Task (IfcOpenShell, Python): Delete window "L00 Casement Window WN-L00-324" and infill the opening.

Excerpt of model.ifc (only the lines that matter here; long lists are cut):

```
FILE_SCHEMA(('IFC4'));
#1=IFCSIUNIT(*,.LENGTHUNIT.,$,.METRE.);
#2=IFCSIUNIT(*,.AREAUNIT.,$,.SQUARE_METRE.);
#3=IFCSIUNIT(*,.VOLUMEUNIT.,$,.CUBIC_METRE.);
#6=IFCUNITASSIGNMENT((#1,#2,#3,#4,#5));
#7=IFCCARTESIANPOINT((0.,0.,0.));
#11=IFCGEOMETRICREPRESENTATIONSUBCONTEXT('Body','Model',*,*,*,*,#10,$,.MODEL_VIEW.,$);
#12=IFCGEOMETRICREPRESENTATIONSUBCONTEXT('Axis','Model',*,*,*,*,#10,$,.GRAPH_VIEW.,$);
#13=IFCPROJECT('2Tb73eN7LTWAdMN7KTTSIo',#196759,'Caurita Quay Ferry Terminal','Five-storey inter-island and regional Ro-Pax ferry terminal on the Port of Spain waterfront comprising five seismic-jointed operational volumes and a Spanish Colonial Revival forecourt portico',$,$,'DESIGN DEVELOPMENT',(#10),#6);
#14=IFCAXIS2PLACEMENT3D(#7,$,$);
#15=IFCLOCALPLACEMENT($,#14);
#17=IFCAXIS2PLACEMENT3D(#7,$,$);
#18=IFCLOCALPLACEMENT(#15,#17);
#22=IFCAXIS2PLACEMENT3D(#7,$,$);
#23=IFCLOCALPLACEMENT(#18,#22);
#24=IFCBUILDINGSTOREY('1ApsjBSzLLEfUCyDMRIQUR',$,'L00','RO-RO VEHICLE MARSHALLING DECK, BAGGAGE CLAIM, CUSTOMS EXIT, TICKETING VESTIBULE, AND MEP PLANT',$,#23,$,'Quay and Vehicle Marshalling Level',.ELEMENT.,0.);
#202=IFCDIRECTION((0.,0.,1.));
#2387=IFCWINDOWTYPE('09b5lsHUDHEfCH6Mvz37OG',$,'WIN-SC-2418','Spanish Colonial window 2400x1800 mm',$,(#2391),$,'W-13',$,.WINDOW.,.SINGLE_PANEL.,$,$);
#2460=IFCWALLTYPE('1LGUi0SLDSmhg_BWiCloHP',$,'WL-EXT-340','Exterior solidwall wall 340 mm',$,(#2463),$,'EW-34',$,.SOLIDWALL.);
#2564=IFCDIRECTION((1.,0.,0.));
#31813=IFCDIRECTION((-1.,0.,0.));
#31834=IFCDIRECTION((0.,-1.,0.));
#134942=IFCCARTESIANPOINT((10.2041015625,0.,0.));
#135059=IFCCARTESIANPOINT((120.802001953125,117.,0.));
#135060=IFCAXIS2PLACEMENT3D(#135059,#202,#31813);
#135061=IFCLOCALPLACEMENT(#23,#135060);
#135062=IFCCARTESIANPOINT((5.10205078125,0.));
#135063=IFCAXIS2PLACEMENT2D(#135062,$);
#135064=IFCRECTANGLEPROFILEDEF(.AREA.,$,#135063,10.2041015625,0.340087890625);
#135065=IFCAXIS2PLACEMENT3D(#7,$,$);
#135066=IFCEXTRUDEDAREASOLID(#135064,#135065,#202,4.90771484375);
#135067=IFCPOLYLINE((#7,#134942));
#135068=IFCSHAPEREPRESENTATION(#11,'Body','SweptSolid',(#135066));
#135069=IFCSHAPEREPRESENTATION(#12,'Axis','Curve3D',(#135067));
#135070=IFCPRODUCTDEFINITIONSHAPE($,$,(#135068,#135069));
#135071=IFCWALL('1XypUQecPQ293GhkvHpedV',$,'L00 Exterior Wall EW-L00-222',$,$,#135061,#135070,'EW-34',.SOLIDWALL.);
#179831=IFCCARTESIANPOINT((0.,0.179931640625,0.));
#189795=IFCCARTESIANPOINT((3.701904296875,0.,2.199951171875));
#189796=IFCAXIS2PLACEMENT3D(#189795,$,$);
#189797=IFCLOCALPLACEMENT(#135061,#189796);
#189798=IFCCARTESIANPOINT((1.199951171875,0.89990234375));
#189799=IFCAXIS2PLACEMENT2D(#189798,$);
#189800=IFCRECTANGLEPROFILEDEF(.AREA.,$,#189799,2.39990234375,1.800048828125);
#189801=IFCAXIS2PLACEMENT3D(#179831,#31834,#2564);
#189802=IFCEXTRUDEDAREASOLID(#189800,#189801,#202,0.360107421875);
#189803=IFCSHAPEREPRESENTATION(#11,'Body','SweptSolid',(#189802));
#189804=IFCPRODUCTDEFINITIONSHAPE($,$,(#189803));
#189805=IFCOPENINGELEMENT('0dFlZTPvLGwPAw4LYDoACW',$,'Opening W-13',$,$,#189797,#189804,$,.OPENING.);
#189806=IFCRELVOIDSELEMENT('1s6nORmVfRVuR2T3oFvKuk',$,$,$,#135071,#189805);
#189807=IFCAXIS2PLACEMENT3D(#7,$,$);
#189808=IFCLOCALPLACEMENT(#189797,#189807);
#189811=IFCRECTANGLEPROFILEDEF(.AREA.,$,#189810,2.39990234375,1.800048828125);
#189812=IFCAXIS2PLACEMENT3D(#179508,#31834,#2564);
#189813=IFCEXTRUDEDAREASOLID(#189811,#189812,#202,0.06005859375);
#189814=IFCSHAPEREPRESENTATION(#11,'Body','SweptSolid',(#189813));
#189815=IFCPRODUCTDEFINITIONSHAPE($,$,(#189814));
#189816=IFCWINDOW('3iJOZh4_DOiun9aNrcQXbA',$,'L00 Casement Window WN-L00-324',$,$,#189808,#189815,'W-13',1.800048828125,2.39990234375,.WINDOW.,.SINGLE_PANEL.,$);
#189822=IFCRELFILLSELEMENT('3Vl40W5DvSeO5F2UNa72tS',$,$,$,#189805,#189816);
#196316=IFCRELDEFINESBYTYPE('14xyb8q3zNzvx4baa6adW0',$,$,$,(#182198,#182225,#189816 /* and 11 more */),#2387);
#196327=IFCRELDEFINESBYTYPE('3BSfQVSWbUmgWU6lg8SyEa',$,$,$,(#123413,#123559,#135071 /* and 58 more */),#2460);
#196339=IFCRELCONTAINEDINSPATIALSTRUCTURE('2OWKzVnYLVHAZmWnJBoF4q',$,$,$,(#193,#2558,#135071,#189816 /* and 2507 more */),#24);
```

```python
import ifcopenshell
import ifcopenshell.api.feature
import ifcopenshell.api.root
import ifcopenshell.geom
import ifcopenshell.util.shape

model = ifcopenshell.open("model.ifc")
settings = ifcopenshell.geom.settings()


def volume(element):
    """Net volume in cubic metres, openings subtracted."""
    shape = ifcopenshell.geom.create_shape(settings, element)
    return ifcopenshell.util.shape.get_volume(shape.geometry)


window = model.by_guid("3iJOZh4_DOiun9aNrcQXbA")
opening = window.FillsVoids[0].RelatingOpeningElement
wall = opening.VoidsElements[0].RelatingBuildingElement
before = volume(wall)

ifcopenshell.api.root.remove_product(model, product=window)
ifcopenshell.api.feature.remove_feature(model, feature=opening)

after = volume(wall)

print(f"wall volume {before:.3f} -> {after:.3f} m3")

model.write("model_rev.ifc")
```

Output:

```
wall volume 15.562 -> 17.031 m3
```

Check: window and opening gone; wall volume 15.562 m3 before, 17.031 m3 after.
